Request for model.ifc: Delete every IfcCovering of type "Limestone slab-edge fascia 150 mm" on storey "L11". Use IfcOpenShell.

First a look at what the model holds.

```python
import ifcopenshell
import ifcopenshell.util.element

model = ifcopenshell.open("model.ifc")
print(model.schema)
storey = next(s for s in model.by_type("IfcBuildingStorey") if s.Name == "L11")
coverings = [e for e in ifcopenshell.util.element.get_decomposition(storey) if e.is_a("IfcCovering")]
seen = {}
for e in coverings:
    element_type = ifcopenshell.util.element.get_type(e)
    name = element_type.Name if element_type not in (None, e) else None
    seen[name] = seen.get(name, 0) + 1
for name, count in sorted(seen.items(), key=str):
    print(count, "x", name)
```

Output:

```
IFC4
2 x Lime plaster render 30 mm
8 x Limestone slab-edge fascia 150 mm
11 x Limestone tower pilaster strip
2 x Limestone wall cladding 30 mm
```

```python
import ifcopenshell
import ifcopenshell.api.root
import ifcopenshell.util.element

model = ifcopenshell.open("model.ifc")

storey = next(s for s in model.by_type("IfcBuildingStorey") if s.Name == "L11")
coverings = [e for e in ifcopenshell.util.element.get_decomposition(storey) if e.is_a("IfcCovering")]
targets = [e for e in coverings if (t := ifcopenshell.util.element.get_type(e)) not in (None, e) and t.Name == "Limestone slab-edge fascia 150 mm"]

for e in targets:
    ifcopenshell.api.root.remove_product(model, product=e)
print(len(targets), "removed")

model.write("model_v2.ifc")
```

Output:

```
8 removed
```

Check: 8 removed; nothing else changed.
